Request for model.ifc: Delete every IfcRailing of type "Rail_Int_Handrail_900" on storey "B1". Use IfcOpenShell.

First a look at what the model holds.

```python
import ifcopenshell
import ifcopenshell.util.element

model = ifcopenshell.open("model.ifc")
print(model.schema)
storey = next(s for s in model.by_type("IfcBuildingStorey") if s.Name == "B1")
railings = [e for e in ifcopenshell.util.element.get_decomposition(storey) if e.is_a("IfcRailing")]
seen = {}
for e in railings:
    element_type = ifcopenshell.util.element.get_type(e)
    name = element_type.Name if element_type not in (None, e) else None
    seen[name] = seen.get(name, 0) + 1
for name, count in sorted(seen.items(), key=str):
    print(count, "x", name)
```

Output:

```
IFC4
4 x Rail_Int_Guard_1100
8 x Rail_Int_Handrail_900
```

```python
import ifcopenshell
import ifcopenshell.api.root
import ifcopenshell.util.element

model = ifcopenshell.open("model.ifc")

storey = next(s for s in model.by_type("IfcBuildingStorey") if s.Name == "B1")
railings = [e for e in ifcopenshell.util.element.get_decomposition(storey) if e.is_a("IfcRailing")]
targets = [e for e in railings if (t := ifcopenshell.util.element.get_type(e)) not in (None, e) and t.Name == "Rail_Int_Handrail_900"]

for e in targets:
    ifcopenshell.api.root.remove_product(model, product=e)
print(len(targets), "removed")

model.write("model_rev.ifc")
```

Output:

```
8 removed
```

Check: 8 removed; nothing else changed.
